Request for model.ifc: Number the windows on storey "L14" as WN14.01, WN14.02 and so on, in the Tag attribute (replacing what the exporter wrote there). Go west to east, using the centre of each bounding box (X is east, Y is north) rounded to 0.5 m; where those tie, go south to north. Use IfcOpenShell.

First a look at what the model holds.

```python
import ifcopenshell
import ifcopenshell.util.element
import ifcopenshell.util.placement

model = ifcopenshell.open("model.ifc")
print(model.schema)
storey = next(s for s in model.by_type("IfcBuildingStorey") if s.Name == "L14")
windows = [e for e in ifcopenshell.util.element.get_decomposition(storey) if e.is_a("IfcWindow")]
for e in sorted(windows, key=lambda e: e.id()):
    origin = ifcopenshell.util.placement.get_local_placement(e.ObjectPlacement)[:3, 3]
    print(e.id(), e.Tag, e.Name, origin.round(2) + 0.0, sep=" | ")
```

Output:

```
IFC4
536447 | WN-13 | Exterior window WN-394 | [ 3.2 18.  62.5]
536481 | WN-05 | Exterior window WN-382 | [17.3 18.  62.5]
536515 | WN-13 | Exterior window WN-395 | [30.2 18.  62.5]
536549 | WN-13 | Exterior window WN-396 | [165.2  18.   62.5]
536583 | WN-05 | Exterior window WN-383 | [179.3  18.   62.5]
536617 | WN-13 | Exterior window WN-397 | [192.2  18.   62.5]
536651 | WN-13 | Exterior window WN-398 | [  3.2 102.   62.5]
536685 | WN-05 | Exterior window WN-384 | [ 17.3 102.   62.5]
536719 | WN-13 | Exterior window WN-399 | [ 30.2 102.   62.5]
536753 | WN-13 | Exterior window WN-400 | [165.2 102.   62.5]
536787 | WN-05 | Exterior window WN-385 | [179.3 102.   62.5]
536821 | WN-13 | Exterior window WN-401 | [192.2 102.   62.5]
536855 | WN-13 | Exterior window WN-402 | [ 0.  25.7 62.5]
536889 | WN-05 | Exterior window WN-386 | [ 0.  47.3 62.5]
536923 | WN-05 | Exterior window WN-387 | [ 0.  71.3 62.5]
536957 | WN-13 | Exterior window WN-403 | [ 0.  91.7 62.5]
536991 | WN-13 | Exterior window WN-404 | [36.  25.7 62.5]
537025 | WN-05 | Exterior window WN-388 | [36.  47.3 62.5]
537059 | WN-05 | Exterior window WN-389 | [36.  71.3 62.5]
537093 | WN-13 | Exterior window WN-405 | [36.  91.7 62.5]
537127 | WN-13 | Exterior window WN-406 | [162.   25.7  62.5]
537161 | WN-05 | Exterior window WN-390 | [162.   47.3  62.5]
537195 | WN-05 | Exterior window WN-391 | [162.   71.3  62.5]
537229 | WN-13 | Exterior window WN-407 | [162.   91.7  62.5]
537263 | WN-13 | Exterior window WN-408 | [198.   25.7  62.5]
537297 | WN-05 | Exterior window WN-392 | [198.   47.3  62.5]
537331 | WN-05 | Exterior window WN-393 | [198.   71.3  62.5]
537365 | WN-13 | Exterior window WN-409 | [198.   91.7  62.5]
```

```python
import ifcopenshell
import ifcopenshell.geom
import ifcopenshell.util.element
import ifcopenshell.util.shape

model = ifcopenshell.open("model.ifc")
settings = ifcopenshell.geom.settings()
settings.set("use-world-coords", True)


def centre(element):
    shape = ifcopenshell.geom.create_shape(settings, element)
    return ifcopenshell.util.shape.get_bbox_centroid(shape.geometry)


storey = next(s for s in model.by_type("IfcBuildingStorey") if s.Name == "L14")
windows = [e for e in ifcopenshell.util.element.get_decomposition(storey) if e.is_a("IfcWindow")]

# Insertion points can sit at a corner or the storey origin, so sort by the geometry (in metres).
centres = {e: centre(e) for e in windows}
windows.sort(key=lambda e: (round(centres[e][0] / 0.5), centres[e][1]))

for i, e in enumerate(windows, start=1):
    number = f"WN14.{i:02d}"
    e.Tag = number
    print(e.id(), number)

model.write("model_updated.ifc")
```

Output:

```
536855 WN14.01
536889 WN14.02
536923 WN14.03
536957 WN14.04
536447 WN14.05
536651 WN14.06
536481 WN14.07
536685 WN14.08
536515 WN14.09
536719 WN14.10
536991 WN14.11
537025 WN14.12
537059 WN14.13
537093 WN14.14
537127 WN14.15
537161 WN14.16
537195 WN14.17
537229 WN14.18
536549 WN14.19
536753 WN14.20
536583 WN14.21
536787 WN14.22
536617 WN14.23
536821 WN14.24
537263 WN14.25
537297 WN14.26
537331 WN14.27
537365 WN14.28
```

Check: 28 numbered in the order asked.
